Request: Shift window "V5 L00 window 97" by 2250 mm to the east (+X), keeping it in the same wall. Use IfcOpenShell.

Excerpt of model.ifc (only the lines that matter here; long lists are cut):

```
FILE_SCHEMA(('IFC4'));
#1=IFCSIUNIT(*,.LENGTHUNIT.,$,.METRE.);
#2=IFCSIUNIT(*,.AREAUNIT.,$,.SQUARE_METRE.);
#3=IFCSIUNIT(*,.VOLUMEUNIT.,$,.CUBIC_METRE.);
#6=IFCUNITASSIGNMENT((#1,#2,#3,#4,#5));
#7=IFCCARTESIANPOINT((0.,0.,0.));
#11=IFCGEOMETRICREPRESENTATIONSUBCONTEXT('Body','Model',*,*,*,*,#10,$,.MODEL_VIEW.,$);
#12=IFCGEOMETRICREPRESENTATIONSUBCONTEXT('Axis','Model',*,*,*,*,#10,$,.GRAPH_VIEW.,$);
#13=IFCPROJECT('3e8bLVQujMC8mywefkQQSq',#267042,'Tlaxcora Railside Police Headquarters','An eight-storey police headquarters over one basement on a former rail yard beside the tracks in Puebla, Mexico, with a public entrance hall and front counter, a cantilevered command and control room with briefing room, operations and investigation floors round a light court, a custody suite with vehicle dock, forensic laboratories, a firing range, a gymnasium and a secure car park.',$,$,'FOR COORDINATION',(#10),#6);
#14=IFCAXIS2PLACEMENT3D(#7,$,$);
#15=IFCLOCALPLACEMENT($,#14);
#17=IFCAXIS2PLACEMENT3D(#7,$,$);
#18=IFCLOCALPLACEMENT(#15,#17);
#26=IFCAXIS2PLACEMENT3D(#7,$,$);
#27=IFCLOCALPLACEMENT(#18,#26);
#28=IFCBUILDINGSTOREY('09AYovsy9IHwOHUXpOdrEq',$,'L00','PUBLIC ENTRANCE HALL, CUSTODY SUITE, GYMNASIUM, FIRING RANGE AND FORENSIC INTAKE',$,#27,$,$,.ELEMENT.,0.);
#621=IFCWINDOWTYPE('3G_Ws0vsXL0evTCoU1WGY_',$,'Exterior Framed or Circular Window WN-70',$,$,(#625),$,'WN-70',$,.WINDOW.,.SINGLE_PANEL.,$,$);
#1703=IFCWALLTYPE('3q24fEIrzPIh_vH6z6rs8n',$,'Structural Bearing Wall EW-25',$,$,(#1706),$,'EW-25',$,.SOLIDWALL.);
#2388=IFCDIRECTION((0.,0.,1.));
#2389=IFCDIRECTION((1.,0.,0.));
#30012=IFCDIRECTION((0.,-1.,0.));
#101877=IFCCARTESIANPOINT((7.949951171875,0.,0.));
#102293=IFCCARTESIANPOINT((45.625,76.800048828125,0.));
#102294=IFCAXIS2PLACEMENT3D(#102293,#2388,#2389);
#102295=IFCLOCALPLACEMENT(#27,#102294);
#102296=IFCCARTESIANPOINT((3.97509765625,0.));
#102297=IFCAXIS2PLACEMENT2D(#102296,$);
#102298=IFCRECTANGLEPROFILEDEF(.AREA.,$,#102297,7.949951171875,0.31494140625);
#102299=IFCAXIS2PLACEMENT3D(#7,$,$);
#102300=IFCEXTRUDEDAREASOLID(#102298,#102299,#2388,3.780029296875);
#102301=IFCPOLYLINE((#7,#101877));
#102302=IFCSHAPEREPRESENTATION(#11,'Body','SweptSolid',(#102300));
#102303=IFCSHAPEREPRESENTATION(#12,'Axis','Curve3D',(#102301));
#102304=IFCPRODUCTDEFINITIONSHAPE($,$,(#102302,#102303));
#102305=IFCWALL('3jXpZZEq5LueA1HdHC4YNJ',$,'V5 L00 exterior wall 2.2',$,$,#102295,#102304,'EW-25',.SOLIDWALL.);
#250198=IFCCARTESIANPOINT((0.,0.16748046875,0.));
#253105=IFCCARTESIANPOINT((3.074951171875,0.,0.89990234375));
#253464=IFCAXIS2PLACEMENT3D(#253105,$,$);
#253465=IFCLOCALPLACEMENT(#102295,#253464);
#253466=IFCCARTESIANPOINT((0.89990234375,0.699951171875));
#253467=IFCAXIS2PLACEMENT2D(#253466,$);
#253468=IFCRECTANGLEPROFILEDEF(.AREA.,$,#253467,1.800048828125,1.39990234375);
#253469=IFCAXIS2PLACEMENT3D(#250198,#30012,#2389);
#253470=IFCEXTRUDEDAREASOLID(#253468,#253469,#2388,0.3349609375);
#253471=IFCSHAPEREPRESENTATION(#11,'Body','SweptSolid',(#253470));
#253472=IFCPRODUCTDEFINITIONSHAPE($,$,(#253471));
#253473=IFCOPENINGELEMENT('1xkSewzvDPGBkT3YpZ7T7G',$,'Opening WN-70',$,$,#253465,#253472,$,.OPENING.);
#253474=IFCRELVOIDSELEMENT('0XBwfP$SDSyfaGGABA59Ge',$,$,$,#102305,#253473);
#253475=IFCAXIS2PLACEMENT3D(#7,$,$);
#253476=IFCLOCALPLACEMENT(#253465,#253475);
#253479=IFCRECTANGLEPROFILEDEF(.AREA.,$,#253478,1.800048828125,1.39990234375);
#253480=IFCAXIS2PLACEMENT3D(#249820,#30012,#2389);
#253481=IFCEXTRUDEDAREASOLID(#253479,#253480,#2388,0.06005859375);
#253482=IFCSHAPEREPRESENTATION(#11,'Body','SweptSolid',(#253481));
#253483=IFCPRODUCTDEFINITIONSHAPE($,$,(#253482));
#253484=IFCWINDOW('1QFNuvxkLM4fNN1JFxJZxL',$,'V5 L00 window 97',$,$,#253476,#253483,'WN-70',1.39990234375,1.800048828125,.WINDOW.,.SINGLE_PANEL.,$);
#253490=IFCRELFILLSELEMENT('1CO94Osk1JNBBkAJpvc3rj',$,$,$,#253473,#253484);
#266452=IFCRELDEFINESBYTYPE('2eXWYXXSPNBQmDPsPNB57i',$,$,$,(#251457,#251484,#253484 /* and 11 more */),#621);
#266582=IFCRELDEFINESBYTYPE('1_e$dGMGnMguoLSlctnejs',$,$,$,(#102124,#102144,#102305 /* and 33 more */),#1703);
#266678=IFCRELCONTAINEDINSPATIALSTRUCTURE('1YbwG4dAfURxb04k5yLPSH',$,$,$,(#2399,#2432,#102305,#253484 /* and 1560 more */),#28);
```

```python
import ifcopenshell
import ifcopenshell.api.geometry
import ifcopenshell.util.placement

model = ifcopenshell.open("model.ifc")

window = model.by_guid("1QFNuvxkLM4fNN1JFxJZxL")
opening = window.FillsVoids[0].RelatingOpeningElement
wall = opening.VoidsElements[0].RelatingBuildingElement

wall_matrix = ifcopenshell.util.placement.get_local_placement(wall.ObjectPlacement)
shift = wall_matrix[:3, 0] * 2.25
before = ifcopenshell.util.placement.get_local_placement(window.ObjectPlacement)[:3, 3].copy()

# The window is placed relative to its opening, so it follows when the opening moves.
matrix = ifcopenshell.util.placement.get_local_placement(opening.ObjectPlacement)
matrix[:3, 3] += shift
ifcopenshell.api.geometry.edit_object_placement(
    model, product=opening, matrix=matrix, is_si=False, should_transform_children=True
)

after = ifcopenshell.util.placement.get_local_placement(window.ObjectPlacement)[:3, 3]
print("window moved by", (after - before).round(3) + 0.0)

model.write("model_updated.ifc")
```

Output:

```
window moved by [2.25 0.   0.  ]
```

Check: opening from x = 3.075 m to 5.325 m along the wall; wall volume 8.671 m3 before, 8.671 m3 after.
